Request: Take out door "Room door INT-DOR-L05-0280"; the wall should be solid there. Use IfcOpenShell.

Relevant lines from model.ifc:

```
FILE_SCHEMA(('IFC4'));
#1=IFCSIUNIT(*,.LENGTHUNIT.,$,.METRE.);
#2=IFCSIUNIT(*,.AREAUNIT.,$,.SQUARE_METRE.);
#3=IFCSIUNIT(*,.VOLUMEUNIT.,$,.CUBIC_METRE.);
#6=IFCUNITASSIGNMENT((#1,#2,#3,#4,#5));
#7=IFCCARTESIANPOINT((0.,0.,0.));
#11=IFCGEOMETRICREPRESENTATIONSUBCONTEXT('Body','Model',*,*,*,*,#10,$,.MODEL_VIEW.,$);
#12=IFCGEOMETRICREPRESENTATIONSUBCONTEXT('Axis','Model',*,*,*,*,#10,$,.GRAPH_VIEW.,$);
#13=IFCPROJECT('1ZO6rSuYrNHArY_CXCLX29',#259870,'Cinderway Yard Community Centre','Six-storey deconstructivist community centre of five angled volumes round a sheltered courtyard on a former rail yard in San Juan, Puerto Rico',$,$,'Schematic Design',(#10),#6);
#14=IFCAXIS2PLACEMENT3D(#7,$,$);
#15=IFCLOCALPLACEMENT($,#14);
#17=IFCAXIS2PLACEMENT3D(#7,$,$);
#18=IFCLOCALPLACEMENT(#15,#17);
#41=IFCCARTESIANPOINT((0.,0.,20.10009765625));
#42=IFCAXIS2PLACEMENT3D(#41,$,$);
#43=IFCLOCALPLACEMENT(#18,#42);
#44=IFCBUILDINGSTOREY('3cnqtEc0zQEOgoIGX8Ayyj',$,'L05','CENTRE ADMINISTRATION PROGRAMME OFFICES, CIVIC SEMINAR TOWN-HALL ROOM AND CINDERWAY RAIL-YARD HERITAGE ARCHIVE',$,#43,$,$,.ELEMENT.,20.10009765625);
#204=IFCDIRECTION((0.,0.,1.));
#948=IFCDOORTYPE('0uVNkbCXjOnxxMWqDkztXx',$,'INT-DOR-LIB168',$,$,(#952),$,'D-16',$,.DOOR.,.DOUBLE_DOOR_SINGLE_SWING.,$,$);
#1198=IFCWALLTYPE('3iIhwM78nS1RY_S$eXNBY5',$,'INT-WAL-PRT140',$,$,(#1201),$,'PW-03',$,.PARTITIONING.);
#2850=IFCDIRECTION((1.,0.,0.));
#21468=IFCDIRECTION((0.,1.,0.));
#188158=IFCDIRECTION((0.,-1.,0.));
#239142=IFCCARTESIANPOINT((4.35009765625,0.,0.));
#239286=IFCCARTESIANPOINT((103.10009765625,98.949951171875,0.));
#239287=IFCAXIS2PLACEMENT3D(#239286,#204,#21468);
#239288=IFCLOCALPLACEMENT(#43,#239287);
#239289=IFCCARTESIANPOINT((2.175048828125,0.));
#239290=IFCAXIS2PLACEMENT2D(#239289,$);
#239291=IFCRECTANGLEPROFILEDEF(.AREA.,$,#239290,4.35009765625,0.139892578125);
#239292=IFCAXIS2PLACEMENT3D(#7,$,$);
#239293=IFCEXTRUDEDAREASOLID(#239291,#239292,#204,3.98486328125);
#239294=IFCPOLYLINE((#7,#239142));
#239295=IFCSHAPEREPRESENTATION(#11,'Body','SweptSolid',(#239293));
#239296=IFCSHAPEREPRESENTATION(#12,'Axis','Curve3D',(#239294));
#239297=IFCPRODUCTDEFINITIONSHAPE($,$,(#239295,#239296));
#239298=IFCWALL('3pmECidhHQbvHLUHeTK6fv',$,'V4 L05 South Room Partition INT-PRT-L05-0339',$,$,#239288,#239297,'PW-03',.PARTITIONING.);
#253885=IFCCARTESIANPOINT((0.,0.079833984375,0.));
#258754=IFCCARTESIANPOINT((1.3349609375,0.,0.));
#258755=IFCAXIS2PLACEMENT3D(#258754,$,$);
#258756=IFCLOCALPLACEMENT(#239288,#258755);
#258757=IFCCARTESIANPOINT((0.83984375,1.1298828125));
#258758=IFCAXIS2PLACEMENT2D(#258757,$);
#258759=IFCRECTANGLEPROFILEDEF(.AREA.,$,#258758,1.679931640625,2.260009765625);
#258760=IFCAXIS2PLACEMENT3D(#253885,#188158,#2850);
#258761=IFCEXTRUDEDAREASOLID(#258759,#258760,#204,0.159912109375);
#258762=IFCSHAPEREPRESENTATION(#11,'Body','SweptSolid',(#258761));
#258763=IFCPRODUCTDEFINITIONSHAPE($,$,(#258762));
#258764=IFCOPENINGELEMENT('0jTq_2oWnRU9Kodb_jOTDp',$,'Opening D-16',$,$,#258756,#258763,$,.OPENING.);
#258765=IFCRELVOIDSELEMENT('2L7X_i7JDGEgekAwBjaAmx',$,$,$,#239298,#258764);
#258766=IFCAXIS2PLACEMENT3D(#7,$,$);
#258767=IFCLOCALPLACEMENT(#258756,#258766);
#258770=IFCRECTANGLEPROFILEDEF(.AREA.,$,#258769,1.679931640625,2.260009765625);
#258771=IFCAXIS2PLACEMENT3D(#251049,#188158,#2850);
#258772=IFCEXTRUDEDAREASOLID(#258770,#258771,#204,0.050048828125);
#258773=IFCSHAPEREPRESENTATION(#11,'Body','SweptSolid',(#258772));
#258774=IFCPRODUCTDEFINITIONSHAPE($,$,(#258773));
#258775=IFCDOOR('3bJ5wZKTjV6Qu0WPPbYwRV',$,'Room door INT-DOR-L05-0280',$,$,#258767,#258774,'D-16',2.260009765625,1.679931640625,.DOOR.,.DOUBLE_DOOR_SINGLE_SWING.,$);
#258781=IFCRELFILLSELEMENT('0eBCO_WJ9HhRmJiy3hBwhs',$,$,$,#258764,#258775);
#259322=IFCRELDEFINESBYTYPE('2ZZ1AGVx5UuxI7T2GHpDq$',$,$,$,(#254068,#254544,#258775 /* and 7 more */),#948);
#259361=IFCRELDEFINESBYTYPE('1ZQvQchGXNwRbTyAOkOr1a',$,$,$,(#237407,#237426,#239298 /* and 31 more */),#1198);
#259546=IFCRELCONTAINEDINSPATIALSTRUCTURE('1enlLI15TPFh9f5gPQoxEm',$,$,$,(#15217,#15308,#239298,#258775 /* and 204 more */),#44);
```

```python
import ifcopenshell
import ifcopenshell.api.feature
import ifcopenshell.api.root
import ifcopenshell.geom
import ifcopenshell.util.shape

model = ifcopenshell.open("model.ifc")
settings = ifcopenshell.geom.settings()


def volume(element):
    """Net volume in cubic metres, openings subtracted."""
    shape = ifcopenshell.geom.create_shape(settings, element)
    return ifcopenshell.util.shape.get_volume(shape.geometry)


door = model.by_id(258775)
opening = door.FillsVoids[0].RelatingOpeningElement
wall = opening.VoidsElements[0].RelatingBuildingElement
before = volume(wall)

ifcopenshell.api.root.remove_product(model, product=door)
ifcopenshell.api.feature.remove_feature(model, feature=opening)

after = volume(wall)

print(f"wall volume {before:.3f} -> {after:.3f} m3")

model.write("model_updated.ifc")
```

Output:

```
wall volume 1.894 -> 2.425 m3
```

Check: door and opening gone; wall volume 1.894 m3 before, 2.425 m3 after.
